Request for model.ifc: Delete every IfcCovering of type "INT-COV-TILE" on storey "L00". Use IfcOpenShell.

First a look at what the model holds.

```python
import ifcopenshell
import ifcopenshell.util.element

model = ifcopenshell.open("model.ifc")
print(model.schema)
storey = next(s for s in model.by_type("IfcBuildingStorey") if s.Name == "L00")
coverings = [e for e in ifcopenshell.util.element.get_decomposition(storey) if e.is_a("IfcCovering")]
seen = {}
for e in coverings:
    element_type = ifcopenshell.util.element.get_type(e)
    name = element_type.Name if element_type not in (None, e) else None
    seen[name] = seen.get(name, 0) + 1
for name, count in sorted(seen.items(), key=str):
    print(count, "x", name)
```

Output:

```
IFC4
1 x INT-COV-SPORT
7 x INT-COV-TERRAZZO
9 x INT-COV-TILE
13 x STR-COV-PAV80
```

```python
import ifcopenshell
import ifcopenshell.api.root
import ifcopenshell.util.element

model = ifcopenshell.open("model.ifc")

storey = next(s for s in model.by_type("IfcBuildingStorey") if s.Name == "L00")
coverings = [e for e in ifcopenshell.util.element.get_decomposition(storey) if e.is_a("IfcCovering")]
targets = [e for e in coverings if (t := ifcopenshell.util.element.get_type(e)) not in (None, e) and t.Name == "INT-COV-TILE"]

for e in targets:
    ifcopenshell.api.root.remove_product(model, product=e)
print(len(targets), "removed")

model.write("model_edited.ifc")
```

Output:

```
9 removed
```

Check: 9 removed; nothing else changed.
